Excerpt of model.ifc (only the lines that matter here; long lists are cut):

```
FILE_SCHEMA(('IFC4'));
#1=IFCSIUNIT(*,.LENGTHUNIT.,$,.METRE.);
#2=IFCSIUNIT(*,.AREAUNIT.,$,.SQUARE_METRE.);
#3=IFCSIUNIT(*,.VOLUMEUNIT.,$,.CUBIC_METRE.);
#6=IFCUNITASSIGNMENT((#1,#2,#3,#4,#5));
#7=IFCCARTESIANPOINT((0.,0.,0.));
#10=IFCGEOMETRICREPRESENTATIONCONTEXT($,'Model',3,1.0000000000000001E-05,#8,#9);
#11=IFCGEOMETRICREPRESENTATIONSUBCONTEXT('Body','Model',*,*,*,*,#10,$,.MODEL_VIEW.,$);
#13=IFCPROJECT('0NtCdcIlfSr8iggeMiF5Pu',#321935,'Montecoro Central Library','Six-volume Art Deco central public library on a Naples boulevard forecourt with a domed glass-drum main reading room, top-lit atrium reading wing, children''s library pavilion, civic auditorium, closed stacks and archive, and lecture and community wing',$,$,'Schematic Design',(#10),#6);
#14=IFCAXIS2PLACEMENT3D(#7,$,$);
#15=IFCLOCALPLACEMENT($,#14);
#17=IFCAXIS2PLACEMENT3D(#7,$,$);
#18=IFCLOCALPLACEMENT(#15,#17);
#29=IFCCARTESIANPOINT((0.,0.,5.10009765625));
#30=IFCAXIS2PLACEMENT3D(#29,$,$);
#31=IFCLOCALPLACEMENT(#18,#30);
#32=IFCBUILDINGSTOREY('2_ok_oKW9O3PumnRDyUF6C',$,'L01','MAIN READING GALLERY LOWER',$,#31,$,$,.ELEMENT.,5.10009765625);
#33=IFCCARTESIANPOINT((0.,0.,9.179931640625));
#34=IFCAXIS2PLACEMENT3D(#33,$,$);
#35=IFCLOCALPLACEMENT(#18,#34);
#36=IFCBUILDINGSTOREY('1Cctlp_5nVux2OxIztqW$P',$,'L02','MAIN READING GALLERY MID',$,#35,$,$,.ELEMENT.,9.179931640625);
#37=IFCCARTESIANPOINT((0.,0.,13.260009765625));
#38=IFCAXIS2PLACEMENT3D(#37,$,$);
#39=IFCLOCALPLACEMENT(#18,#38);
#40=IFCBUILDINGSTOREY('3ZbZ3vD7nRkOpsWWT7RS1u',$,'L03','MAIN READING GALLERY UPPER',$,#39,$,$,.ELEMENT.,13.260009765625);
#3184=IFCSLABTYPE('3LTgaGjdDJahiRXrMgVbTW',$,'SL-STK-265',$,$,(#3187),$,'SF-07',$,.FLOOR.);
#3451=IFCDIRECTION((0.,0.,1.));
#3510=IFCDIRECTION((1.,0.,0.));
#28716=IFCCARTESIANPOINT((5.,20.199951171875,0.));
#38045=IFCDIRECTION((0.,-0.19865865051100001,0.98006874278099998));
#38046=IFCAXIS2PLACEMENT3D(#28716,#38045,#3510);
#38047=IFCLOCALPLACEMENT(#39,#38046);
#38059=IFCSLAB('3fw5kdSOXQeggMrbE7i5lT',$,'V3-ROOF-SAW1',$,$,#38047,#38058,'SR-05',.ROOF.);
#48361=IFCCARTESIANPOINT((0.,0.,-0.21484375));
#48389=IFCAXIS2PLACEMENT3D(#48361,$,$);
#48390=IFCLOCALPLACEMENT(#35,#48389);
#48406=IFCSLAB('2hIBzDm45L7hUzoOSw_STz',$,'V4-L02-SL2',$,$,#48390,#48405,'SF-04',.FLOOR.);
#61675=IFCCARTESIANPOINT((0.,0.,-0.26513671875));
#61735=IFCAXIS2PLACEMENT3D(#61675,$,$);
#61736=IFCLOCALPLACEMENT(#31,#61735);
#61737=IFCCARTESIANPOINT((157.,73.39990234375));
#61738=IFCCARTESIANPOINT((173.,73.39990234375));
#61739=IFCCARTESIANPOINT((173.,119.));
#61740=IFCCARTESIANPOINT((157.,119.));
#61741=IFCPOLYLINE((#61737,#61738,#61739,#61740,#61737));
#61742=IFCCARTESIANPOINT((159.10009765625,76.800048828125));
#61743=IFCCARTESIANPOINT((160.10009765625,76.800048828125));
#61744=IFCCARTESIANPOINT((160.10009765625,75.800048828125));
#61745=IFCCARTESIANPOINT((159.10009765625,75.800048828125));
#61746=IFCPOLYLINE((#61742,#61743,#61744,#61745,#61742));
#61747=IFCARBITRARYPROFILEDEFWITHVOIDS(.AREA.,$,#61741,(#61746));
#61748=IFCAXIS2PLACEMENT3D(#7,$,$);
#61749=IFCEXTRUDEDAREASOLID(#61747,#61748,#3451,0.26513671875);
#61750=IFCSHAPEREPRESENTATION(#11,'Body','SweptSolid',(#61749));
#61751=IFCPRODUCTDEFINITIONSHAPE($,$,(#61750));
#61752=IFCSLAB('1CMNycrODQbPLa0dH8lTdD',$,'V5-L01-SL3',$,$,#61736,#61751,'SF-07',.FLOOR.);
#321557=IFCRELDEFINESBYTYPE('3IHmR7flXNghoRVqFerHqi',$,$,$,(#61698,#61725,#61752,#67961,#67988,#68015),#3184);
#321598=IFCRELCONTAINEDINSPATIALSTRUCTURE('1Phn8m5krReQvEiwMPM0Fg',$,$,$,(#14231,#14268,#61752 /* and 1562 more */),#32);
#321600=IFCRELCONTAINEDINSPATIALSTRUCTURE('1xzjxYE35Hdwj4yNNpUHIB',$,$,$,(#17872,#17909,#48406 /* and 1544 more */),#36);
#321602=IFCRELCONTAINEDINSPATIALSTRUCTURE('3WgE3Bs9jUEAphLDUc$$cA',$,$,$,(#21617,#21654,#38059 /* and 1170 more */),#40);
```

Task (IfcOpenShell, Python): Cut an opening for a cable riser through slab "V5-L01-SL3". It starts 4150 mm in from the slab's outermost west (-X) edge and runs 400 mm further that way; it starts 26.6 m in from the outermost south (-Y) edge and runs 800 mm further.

```python
import numpy as np
import ifcopenshell
import ifcopenshell.api.feature
import ifcopenshell.api.geometry
import ifcopenshell.api.root
import ifcopenshell.geom
import ifcopenshell.util.placement
import ifcopenshell.util.representation
import ifcopenshell.util.shape
import ifcopenshell.util.unit

model = ifcopenshell.open("model.ifc")
unit_scale = ifcopenshell.util.unit.calculate_unit_scale(model)
settings = ifcopenshell.geom.settings()


def volume(element):
    """Net volume in cubic metres, openings subtracted."""
    shape = ifcopenshell.geom.create_shape(settings, element)
    return ifcopenshell.util.shape.get_volume(shape.geometry)


slab = model.by_guid("1CMNycrODQbPLa0dH8lTdD")
before = volume(slab)

# Extent in the slab's own axes, in metres. The edges named are its -X and -Y sides.
slab_shape = ifcopenshell.geom.create_shape(settings, slab)
vertices = ifcopenshell.util.shape.get_vertices(slab_shape.geometry)
x_min, y_min, bottom = vertices.min(axis=0)
top = vertices[:, 2].max()

opening = ifcopenshell.api.root.create_entity(model, ifc_class="IfcOpeningElement", name="Cable riser opening", predefined_type="OPENING")
context = ifcopenshell.util.representation.get_context(model, "Model", "Body", "MODEL_VIEW")
width, depth = 0.4, 0.8
outline = [(0.0, 0.0), (width, 0.0), (width, depth), (0.0, depth), (0.0, 0.0)]
# Overshoot both faces by 50 mm so the cut is clean.
shape = ifcopenshell.api.geometry.add_slab_representation(
    model, context=context, depth=top - bottom + 0.1, polyline=outline
)
ifcopenshell.api.geometry.assign_representation(model, product=opening, representation=shape)

matrix = ifcopenshell.util.placement.get_local_placement(slab.ObjectPlacement)
matrix[:, 3] = matrix @ np.append(np.array([x_min + 4.15, y_min + 26.6, bottom - 0.05]) / unit_scale, 1.0)
ifcopenshell.api.geometry.edit_object_placement(model, product=opening, matrix=matrix, is_si=False)
ifcopenshell.api.feature.add_feature(model, feature=opening, element=slab)

after = volume(slab)

print(f"slab volume {before:.3f} -> {after:.3f} m3")

model.write("model_v2.ifc")
```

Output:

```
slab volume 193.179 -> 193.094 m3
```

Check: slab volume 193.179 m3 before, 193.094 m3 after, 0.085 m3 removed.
